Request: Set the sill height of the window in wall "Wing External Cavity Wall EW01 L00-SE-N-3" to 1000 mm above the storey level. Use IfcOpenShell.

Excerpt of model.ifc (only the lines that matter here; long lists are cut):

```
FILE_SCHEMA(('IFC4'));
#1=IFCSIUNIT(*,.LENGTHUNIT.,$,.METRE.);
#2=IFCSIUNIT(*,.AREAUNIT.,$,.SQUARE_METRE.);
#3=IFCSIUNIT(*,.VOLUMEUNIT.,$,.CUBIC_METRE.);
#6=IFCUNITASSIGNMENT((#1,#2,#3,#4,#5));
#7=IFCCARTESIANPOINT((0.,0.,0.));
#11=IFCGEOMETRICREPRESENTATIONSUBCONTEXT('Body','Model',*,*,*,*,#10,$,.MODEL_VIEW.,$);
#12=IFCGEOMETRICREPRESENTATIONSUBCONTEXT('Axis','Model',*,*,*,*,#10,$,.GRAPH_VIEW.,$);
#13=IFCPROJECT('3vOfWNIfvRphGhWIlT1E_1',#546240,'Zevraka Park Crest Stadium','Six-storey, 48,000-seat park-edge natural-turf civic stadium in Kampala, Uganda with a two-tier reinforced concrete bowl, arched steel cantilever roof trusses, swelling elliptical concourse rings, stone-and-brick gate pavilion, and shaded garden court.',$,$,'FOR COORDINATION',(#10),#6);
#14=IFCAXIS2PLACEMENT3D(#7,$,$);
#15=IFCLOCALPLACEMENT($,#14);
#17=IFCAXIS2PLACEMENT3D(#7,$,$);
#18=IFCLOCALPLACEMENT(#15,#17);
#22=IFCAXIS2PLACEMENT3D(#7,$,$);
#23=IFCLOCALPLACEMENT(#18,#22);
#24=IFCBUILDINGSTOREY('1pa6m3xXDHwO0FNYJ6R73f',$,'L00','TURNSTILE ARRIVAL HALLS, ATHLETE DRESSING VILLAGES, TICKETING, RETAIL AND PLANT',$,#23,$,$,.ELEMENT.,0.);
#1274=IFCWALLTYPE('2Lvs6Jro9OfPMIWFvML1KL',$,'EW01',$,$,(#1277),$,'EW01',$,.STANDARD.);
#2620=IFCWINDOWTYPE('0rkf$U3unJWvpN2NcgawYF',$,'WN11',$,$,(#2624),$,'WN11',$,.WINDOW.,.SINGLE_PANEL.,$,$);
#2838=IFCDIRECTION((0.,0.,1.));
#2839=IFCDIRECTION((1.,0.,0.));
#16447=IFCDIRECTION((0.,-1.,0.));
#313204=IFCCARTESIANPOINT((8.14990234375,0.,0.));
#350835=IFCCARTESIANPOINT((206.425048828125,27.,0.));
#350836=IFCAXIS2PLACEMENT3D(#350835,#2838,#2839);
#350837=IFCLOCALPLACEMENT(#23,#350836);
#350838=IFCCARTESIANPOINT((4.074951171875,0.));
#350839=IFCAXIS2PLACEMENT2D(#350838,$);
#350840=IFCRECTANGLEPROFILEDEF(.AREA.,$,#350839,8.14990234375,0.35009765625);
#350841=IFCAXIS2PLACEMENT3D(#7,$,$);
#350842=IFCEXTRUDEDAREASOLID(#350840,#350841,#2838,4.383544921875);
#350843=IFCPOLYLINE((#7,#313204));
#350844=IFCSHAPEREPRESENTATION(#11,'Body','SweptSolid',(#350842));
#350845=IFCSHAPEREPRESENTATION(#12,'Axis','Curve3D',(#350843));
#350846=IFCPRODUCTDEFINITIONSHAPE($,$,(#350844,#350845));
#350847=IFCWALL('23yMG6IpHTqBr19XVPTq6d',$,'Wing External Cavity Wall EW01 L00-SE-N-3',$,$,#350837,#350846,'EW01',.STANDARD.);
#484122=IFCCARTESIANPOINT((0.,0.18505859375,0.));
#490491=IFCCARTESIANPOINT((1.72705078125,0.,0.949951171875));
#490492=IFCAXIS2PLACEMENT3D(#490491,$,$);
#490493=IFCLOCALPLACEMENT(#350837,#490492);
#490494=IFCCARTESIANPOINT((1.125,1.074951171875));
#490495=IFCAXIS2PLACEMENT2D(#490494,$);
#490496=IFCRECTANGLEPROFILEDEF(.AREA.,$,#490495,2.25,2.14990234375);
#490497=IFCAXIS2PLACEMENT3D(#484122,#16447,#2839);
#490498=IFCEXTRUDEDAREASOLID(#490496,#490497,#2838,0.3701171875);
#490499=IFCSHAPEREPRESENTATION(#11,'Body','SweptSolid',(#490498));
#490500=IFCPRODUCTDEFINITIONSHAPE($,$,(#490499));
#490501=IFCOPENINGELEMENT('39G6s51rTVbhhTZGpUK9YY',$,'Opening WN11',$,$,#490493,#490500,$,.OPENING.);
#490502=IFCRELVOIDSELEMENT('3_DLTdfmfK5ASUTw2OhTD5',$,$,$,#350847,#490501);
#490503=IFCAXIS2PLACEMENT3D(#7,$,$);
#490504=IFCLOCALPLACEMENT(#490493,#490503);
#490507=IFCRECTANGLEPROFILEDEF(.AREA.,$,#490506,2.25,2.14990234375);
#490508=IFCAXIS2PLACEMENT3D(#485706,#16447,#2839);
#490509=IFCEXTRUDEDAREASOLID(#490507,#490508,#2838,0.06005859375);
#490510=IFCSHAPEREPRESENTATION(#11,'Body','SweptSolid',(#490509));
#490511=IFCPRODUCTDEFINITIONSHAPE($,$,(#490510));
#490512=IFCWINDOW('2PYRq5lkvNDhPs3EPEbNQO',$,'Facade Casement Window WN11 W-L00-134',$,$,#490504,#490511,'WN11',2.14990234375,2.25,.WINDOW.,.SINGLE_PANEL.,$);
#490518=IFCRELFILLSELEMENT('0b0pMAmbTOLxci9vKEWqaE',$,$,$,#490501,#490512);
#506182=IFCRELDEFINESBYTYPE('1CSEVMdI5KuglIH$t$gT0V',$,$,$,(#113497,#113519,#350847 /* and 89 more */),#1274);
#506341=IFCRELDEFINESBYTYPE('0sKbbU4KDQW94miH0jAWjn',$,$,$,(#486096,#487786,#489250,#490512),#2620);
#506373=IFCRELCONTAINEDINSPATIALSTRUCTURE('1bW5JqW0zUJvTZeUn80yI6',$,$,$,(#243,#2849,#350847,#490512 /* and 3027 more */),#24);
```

```python
import numpy as np
import ifcopenshell
import ifcopenshell.api.geometry
import ifcopenshell.geom
import ifcopenshell.util.element
import ifcopenshell.util.placement
import ifcopenshell.util.shape
import ifcopenshell.util.unit

model = ifcopenshell.open("model.ifc")
unit_scale = ifcopenshell.util.unit.calculate_unit_scale(model)

window = model.by_id(490512)
opening = window.FillsVoids[0].RelatingOpeningElement
storey = ifcopenshell.util.element.get_container(window, ifc_class="IfcBuildingStorey")
level = ifcopenshell.util.placement.get_local_placement(storey.ObjectPlacement)[2, 3]

# The opening's origin need not be at the sill, so measure its lowest point.
shape = ifcopenshell.geom.create_shape(ifcopenshell.geom.settings(), opening)
bottom = ifcopenshell.util.shape.get_shape_bottom_elevation(shape, shape.geometry) / unit_scale
dz = level + 1 / unit_scale - bottom

shift = np.array([0.0, 0.0, dz])
# The window is placed relative to its opening, so it follows when the opening moves.
matrix = ifcopenshell.util.placement.get_local_placement(opening.ObjectPlacement)
matrix[:3, 3] += shift
ifcopenshell.api.geometry.edit_object_placement(
    model, product=opening, matrix=matrix, is_si=False, should_transform_children=True
)

print(f"moved by {dz * unit_scale:+.3f} m")

model.write("model_updated.ifc")
```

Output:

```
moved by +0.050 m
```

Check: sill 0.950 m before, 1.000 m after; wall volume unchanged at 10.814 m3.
